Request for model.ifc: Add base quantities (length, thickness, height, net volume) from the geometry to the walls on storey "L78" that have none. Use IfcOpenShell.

First a look at what the model holds.

```python
import ifcopenshell
import ifcopenshell.util.element
import ifcopenshell.util.unit

model = ifcopenshell.open("model.ifc")
print(model.schema)
for unit_type in ("LENGTHUNIT", "AREAUNIT", "VOLUMEUNIT"):
    print(unit_type, ifcopenshell.util.unit.calculate_unit_scale(model, unit_type))
storey = next(s for s in model.by_type("IfcBuildingStorey") if s.Name == "L78")
walls = [e for e in ifcopenshell.util.element.get_decomposition(storey) if e.is_a("IfcWall")]
for e in sorted(walls, key=lambda e: e.id()):
    print(e.id(), e.is_a(), e.Name, list(ifcopenshell.util.element.get_psets(e, qtos_only=True)), sep=" | ")
```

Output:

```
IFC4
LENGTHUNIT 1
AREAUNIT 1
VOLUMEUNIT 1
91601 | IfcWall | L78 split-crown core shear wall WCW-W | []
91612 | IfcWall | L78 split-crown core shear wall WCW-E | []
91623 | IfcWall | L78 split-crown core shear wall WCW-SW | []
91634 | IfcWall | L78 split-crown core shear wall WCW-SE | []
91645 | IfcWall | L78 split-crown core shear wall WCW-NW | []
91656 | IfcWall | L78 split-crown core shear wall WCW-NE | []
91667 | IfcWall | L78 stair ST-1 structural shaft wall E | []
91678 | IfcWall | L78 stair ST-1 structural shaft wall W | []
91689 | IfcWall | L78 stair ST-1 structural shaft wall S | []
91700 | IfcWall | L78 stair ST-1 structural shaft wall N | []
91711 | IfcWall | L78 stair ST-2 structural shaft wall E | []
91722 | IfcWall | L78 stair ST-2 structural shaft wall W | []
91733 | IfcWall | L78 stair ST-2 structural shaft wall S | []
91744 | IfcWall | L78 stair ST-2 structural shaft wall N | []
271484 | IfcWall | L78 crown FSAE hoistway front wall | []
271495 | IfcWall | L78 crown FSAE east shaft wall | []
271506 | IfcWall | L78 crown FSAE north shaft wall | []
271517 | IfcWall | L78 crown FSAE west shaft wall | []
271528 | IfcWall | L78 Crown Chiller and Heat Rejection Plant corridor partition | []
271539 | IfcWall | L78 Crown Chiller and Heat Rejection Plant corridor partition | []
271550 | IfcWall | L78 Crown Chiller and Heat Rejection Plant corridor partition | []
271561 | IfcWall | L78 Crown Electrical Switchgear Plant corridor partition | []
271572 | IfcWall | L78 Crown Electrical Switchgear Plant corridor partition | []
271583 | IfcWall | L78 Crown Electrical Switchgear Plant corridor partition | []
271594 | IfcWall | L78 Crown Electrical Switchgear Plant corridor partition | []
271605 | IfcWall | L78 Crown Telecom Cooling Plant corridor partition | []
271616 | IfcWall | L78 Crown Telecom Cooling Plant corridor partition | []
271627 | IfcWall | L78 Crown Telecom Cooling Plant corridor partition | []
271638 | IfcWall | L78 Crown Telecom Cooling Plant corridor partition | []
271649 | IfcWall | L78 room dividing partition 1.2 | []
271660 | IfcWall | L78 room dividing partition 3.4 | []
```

```python
import ifcopenshell
import ifcopenshell.api.pset
import ifcopenshell.geom
import ifcopenshell.util.element
import ifcopenshell.util.shape
import ifcopenshell.util.unit

model = ifcopenshell.open("model.ifc")
unit_scale = ifcopenshell.util.unit.calculate_unit_scale(model)
volume_scale = ifcopenshell.util.unit.calculate_unit_scale(model, "VOLUMEUNIT")
settings = ifcopenshell.geom.settings()

storey = next(s for s in model.by_type("IfcBuildingStorey") if s.Name == "L78")
walls = [e for e in ifcopenshell.util.element.get_decomposition(storey) if e.is_a("IfcWall")]

for e in sorted(walls, key=lambda e: e.id()):
    if ifcopenshell.util.element.get_psets(e, qtos_only=True, should_inherit=False):
        continue
    # Geometry comes back in metres, in the element's own axes.
    shape = ifcopenshell.geom.create_shape(settings, e)
    values = {
        "Length": ifcopenshell.util.shape.get_x(shape.geometry) / unit_scale,
        "Width": ifcopenshell.util.shape.get_y(shape.geometry) / unit_scale,
        "Height": ifcopenshell.util.shape.get_z(shape.geometry) / unit_scale,
        "NetVolume": ifcopenshell.util.shape.get_volume(shape.geometry) / volume_scale,
    }
    qto = ifcopenshell.api.pset.add_qto(model, product=e, name="Qto_WallBaseQuantities")
    ifcopenshell.api.pset.edit_qto(model, qto=qto, properties=values)
    print(e.id(), {k: round(v, 3) for k, v in values.items()})

model.write("model-out.ifc")
```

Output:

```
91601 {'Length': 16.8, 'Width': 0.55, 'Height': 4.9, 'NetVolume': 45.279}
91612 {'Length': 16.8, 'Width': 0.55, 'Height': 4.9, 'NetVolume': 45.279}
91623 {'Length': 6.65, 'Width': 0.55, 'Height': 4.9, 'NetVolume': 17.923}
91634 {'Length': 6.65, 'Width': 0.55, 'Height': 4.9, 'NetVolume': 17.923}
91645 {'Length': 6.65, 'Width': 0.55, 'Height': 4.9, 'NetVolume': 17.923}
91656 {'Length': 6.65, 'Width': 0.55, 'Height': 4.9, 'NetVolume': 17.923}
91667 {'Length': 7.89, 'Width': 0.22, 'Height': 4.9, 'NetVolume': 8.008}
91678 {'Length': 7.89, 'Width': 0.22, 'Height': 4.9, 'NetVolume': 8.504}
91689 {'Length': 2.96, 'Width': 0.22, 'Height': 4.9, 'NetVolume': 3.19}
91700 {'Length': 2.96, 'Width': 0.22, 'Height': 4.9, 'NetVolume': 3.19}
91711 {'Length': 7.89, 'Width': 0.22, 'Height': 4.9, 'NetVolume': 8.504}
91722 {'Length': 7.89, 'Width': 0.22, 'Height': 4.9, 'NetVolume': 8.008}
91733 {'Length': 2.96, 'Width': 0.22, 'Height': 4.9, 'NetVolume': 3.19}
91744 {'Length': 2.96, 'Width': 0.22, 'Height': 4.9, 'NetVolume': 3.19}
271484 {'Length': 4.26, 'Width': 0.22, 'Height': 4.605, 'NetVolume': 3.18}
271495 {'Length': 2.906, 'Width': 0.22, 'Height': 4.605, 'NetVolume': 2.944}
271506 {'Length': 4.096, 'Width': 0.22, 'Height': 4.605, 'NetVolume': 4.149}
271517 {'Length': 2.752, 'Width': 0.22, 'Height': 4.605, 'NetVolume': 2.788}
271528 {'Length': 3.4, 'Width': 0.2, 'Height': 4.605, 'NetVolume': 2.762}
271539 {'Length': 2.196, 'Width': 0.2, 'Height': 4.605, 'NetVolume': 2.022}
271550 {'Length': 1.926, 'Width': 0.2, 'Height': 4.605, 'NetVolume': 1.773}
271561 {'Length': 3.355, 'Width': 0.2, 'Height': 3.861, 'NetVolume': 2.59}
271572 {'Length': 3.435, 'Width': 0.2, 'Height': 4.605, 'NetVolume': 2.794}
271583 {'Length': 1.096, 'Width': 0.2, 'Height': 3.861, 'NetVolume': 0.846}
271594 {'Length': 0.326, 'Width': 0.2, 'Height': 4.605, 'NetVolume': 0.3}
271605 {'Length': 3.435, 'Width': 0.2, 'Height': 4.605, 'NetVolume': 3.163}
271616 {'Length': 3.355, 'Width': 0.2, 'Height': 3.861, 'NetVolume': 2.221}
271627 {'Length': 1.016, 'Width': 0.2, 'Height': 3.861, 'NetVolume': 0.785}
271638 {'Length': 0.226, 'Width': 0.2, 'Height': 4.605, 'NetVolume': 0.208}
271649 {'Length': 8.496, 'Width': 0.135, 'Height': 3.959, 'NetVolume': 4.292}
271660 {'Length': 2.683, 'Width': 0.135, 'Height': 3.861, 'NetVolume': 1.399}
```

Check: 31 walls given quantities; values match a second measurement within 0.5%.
